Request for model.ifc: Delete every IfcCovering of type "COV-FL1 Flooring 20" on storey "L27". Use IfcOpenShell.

First a look at what the model holds.

```python
import ifcopenshell
import ifcopenshell.util.element

model = ifcopenshell.open("model.ifc")
print(model.schema)
storey = next(s for s in model.by_type("IfcBuildingStorey") if s.Name == "L27")
coverings = [e for e in ifcopenshell.util.element.get_decomposition(storey) if e.is_a("IfcCovering")]
seen = {}
for e in coverings:
    element_type = ifcopenshell.util.element.get_type(e)
    name = element_type.Name if element_type not in (None, e) else None
    seen[name] = seen.get(name, 0) + 1
for name, count in sorted(seen.items(), key=str):
    print(count, "x", name)
```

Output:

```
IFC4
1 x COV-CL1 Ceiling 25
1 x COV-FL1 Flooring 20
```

```python
import ifcopenshell
import ifcopenshell.api.root
import ifcopenshell.util.element

model = ifcopenshell.open("model.ifc")

storey = next(s for s in model.by_type("IfcBuildingStorey") if s.Name == "L27")
coverings = [e for e in ifcopenshell.util.element.get_decomposition(storey) if e.is_a("IfcCovering")]
targets = [e for e in coverings if (t := ifcopenshell.util.element.get_type(e)) not in (None, e) and t.Name == "COV-FL1 Flooring 20"]

for e in targets:
    ifcopenshell.api.root.remove_product(model, product=e)
print(len(targets), "removed")

model.write("model_rev.ifc")
```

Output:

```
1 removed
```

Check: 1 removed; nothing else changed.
